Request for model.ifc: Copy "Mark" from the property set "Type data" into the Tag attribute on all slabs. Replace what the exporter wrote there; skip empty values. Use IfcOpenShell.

First a look at what the model holds.

```python
import ifcopenshell
import ifcopenshell.util.element

model = ifcopenshell.open("model.ifc")
print(model.schema)
slabs = model.by_type("IfcSlab")
print(len(slabs), "slabs")
for e in slabs[:8]:
    source = ifcopenshell.util.element.get_pset(e, "Type data", "Mark")
    target = e.Tag
    print(e.id(), repr(source), repr(target), sep=" | ")
```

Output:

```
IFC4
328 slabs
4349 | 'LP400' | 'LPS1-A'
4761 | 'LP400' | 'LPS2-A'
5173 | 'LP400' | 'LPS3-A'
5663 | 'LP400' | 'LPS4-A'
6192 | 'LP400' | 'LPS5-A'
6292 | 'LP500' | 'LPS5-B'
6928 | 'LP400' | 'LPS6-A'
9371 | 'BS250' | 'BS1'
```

```python
import ifcopenshell
import ifcopenshell.util.element

model = ifcopenshell.open("model.ifc")

count = 0
for e in model.by_type("IfcSlab"):
    value = ifcopenshell.util.element.get_pset(e, "Type data", "Mark")
    current = e.Tag
    if not value or not value.strip() or current == value:
        continue
    e.Tag = value
    count += 1

print(count, "slabs updated")

model.write("model_rev.ifc")
```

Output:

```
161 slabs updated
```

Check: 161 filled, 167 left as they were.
